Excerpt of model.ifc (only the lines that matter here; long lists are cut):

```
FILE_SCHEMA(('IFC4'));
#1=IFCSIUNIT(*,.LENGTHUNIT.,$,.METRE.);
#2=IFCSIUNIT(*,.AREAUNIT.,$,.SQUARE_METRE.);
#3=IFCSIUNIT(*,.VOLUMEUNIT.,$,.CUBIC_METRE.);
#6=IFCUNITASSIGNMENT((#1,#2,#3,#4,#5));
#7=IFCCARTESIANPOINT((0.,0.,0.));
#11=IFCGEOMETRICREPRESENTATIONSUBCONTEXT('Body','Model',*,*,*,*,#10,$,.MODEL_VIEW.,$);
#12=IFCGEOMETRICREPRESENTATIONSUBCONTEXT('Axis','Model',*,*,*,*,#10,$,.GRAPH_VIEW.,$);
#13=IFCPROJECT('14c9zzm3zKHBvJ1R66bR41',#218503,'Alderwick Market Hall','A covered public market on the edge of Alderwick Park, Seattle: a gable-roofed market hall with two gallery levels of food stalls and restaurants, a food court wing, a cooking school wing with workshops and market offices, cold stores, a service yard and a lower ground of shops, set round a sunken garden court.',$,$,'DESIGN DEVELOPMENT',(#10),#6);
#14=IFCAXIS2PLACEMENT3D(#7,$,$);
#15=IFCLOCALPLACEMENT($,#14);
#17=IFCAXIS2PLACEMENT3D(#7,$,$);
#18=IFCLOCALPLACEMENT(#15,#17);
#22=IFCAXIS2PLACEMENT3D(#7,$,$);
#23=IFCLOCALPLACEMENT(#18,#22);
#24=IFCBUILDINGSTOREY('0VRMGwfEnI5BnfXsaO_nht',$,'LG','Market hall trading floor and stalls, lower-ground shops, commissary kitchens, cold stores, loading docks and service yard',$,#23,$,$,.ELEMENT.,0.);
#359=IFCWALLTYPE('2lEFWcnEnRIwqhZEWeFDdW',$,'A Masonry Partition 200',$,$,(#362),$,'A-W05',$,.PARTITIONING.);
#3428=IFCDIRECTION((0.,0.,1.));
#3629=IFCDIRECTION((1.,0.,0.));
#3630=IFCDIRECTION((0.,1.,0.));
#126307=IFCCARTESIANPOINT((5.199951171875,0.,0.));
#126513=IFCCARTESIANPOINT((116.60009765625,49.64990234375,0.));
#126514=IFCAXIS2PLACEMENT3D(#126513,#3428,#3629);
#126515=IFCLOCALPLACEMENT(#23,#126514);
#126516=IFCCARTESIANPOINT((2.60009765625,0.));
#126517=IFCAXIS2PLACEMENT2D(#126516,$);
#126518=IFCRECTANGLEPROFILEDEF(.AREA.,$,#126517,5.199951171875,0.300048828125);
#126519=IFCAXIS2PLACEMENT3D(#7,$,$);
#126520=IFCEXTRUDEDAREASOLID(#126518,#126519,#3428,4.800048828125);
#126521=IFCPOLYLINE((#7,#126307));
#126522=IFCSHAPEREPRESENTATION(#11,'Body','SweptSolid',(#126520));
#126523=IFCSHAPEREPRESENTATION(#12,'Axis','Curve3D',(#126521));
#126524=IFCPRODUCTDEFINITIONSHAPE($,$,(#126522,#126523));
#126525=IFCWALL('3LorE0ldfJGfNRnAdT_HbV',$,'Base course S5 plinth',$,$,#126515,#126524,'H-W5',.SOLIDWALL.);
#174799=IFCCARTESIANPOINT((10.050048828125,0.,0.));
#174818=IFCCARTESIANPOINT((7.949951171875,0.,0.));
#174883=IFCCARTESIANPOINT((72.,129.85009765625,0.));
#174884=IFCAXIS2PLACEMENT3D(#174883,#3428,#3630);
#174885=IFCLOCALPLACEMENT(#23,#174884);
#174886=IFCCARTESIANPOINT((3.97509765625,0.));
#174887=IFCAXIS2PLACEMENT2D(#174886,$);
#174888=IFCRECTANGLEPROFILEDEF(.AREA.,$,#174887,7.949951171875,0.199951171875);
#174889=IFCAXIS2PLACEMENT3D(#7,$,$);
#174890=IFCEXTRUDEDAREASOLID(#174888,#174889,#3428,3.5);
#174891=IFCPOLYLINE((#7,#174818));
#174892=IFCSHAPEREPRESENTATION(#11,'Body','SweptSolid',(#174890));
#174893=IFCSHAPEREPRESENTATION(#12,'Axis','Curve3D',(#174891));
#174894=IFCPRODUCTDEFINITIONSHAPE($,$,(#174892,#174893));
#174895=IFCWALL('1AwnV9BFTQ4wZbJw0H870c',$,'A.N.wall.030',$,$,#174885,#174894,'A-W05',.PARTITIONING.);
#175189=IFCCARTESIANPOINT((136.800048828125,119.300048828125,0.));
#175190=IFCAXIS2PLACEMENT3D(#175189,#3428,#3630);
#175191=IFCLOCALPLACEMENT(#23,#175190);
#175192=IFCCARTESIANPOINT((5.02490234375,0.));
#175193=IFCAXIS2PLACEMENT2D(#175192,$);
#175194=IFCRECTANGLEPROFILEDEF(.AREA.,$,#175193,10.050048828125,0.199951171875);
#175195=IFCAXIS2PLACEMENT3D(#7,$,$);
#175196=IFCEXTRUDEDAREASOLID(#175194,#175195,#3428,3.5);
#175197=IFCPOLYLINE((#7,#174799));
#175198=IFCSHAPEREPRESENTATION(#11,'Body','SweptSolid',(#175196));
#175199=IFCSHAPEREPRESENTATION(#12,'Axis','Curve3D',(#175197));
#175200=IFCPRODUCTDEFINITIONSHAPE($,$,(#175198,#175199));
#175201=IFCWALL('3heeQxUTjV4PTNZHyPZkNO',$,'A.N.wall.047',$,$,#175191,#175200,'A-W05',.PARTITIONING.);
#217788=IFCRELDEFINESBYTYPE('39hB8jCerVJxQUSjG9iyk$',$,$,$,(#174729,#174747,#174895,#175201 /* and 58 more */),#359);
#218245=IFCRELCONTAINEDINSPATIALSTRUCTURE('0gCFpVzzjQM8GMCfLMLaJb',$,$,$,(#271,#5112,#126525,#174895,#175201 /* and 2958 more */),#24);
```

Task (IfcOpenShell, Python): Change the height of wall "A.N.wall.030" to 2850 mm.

```python
import ifcopenshell
import ifcopenshell.geom
import ifcopenshell.util.representation
import ifcopenshell.util.shape
import ifcopenshell.util.unit

model = ifcopenshell.open("model.ifc")
unit_scale = ifcopenshell.util.unit.calculate_unit_scale(model)
settings = ifcopenshell.geom.settings()


def volume(element):
    """Net volume in cubic metres, openings subtracted."""
    shape = ifcopenshell.geom.create_shape(settings, element)
    return ifcopenshell.util.shape.get_volume(shape.geometry)


wall = model.by_id(174895)
before = volume(wall)

body = ifcopenshell.util.representation.get_representation(wall, "Model", "Body")
solid = body.Items[0]
old_height = solid.Depth
solid.Depth = 2.85 / unit_scale
after = volume(wall)

print(f"height {old_height:g} -> {solid.Depth:g}, volume {before:.3f} -> {after:.3f} m3")

model.write("model_updated.ifc")
```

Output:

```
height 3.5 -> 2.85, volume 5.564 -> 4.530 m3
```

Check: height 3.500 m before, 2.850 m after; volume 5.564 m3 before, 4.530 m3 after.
